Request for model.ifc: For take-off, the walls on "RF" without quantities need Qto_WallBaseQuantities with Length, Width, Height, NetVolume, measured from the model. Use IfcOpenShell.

First a look at what the model holds.

```python
import ifcopenshell
import ifcopenshell.util.element
import ifcopenshell.util.unit

model = ifcopenshell.open("model.ifc")
print(model.schema)
for unit_type in ("LENGTHUNIT", "AREAUNIT", "VOLUMEUNIT"):
    print(unit_type, ifcopenshell.util.unit.calculate_unit_scale(model, unit_type))
storey = next(s for s in model.by_type("IfcBuildingStorey") if s.Name == "RF")
walls = [e for e in ifcopenshell.util.element.get_decomposition(storey) if e.is_a("IfcWall")]
for e in sorted(walls, key=lambda e: e.id()):
    print(e.id(), e.is_a(), e.Name, list(ifcopenshell.util.element.get_psets(e, qtos_only=True)), sep=" | ")
```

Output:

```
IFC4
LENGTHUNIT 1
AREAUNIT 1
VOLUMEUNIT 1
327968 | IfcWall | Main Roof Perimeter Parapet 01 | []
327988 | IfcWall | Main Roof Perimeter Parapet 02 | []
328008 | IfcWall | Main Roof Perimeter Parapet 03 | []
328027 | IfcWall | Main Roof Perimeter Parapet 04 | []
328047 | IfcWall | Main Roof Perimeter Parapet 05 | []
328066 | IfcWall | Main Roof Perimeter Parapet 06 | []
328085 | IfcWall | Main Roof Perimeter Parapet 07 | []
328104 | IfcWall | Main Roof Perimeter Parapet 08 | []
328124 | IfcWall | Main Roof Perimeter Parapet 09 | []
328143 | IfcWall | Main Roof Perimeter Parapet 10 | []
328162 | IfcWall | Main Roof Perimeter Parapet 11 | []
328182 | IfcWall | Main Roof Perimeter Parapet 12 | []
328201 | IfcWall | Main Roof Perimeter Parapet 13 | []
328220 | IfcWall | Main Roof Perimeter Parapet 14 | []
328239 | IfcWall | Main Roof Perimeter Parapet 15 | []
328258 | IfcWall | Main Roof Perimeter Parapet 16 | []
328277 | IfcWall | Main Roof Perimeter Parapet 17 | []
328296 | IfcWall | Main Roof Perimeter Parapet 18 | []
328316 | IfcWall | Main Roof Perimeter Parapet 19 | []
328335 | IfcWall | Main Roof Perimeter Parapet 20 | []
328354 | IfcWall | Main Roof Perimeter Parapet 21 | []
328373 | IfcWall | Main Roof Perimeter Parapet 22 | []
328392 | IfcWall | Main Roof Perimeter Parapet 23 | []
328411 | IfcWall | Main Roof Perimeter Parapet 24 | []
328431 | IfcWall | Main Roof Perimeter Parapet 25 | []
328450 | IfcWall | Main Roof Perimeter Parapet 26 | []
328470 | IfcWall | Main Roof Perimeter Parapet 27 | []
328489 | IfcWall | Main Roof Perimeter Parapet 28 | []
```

```python
import ifcopenshell
import ifcopenshell.api.pset
import ifcopenshell.geom
import ifcopenshell.util.element
import ifcopenshell.util.shape
import ifcopenshell.util.unit

model = ifcopenshell.open("model.ifc")
unit_scale = ifcopenshell.util.unit.calculate_unit_scale(model)
volume_scale = ifcopenshell.util.unit.calculate_unit_scale(model, "VOLUMEUNIT")
settings = ifcopenshell.geom.settings()

storey = next(s for s in model.by_type("IfcBuildingStorey") if s.Name == "RF")
walls = [e for e in ifcopenshell.util.element.get_decomposition(storey) if e.is_a("IfcWall")]

for e in sorted(walls, key=lambda e: e.id()):
    if ifcopenshell.util.element.get_psets(e, qtos_only=True, should_inherit=False):
        continue
    # Geometry comes back in metres, in the element's own axes.
    shape = ifcopenshell.geom.create_shape(settings, e)
    values = {
        "Length": ifcopenshell.util.shape.get_x(shape.geometry) / unit_scale,
        "Width": ifcopenshell.util.shape.get_y(shape.geometry) / unit_scale,
        "Height": ifcopenshell.util.shape.get_z(shape.geometry) / unit_scale,
        "NetVolume": ifcopenshell.util.shape.get_volume(shape.geometry) / volume_scale,
    }
    qto = ifcopenshell.api.pset.add_qto(model, product=e, name="Qto_WallBaseQuantities")
    ifcopenshell.api.pset.edit_qto(model, qto=qto, properties=values)
    print(e.id(), {k: round(v, 3) for k, v in values.items()})

model.write("model_v2.ifc")
```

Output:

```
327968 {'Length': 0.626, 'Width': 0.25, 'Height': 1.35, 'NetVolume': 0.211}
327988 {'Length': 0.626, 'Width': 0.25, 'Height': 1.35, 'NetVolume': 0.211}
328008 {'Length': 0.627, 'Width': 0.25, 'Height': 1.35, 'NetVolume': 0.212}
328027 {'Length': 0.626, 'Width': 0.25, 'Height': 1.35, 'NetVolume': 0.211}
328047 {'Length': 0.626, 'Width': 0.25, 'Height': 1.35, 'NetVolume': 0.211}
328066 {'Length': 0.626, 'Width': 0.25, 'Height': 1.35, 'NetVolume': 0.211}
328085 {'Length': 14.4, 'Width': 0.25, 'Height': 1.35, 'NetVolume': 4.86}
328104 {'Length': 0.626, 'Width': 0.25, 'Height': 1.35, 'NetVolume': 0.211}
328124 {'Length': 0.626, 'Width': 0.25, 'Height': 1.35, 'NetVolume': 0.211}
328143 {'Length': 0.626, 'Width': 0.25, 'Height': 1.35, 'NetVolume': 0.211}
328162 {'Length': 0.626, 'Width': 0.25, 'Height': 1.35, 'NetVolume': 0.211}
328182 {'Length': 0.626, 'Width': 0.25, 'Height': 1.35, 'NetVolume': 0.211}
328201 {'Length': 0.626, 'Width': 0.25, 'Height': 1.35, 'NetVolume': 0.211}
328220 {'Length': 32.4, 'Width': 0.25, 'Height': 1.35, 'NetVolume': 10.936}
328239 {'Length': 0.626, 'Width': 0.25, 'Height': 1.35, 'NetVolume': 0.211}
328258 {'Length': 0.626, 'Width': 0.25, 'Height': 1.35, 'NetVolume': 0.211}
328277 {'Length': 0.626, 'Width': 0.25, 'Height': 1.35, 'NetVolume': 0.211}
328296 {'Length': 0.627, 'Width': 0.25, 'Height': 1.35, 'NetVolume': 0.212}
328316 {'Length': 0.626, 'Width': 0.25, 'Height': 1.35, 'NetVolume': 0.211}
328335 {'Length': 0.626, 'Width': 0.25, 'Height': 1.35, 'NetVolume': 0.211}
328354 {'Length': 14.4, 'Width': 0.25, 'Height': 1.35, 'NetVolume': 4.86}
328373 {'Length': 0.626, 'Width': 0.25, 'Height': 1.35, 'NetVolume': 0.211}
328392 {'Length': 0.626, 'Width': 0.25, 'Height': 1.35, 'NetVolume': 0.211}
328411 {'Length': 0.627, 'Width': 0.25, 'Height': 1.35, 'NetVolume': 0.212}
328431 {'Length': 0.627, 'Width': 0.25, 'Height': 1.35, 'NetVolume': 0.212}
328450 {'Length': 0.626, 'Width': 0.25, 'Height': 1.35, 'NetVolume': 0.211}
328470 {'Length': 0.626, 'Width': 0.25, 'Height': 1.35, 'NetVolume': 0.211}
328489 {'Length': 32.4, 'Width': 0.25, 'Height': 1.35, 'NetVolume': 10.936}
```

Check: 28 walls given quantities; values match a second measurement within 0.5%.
